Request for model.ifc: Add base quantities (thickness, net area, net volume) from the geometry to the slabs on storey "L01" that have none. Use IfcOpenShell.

First a look at what the model holds.

```python
import ifcopenshell
import ifcopenshell.util.element
import ifcopenshell.util.unit

model = ifcopenshell.open("model.ifc")
print(model.schema)
for unit_type in ("LENGTHUNIT", "AREAUNIT", "VOLUMEUNIT"):
    print(unit_type, ifcopenshell.util.unit.calculate_unit_scale(model, unit_type))
storey = next(s for s in model.by_type("IfcBuildingStorey") if s.Name == "L01")
slabs = [e for e in ifcopenshell.util.element.get_decomposition(storey) if e.is_a("IfcSlab")]
for e in sorted(slabs, key=lambda e: e.id()):
    print(e.id(), e.is_a(), e.Name, list(ifcopenshell.util.element.get_psets(e, qtos_only=True)), sep=" | ")
```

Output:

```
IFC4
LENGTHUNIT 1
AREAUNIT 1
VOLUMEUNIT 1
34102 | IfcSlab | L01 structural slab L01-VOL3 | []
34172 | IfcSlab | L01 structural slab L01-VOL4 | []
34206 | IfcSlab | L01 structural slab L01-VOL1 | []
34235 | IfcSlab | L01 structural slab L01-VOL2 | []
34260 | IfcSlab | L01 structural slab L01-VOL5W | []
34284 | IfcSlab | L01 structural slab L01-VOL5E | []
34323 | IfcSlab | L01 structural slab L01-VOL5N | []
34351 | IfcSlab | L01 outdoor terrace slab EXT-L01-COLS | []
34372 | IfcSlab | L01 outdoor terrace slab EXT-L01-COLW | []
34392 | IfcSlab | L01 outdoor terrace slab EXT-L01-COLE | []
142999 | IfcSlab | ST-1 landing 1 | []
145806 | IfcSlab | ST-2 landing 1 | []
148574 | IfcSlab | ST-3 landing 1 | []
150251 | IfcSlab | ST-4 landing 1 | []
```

```python
import ifcopenshell
import ifcopenshell.api.pset
import ifcopenshell.geom
import ifcopenshell.util.element
import ifcopenshell.util.shape
import ifcopenshell.util.unit

model = ifcopenshell.open("model.ifc")
unit_scale = ifcopenshell.util.unit.calculate_unit_scale(model)
area_scale = ifcopenshell.util.unit.calculate_unit_scale(model, "AREAUNIT")
volume_scale = ifcopenshell.util.unit.calculate_unit_scale(model, "VOLUMEUNIT")
settings = ifcopenshell.geom.settings()

storey = next(s for s in model.by_type("IfcBuildingStorey") if s.Name == "L01")
slabs = [e for e in ifcopenshell.util.element.get_decomposition(storey) if e.is_a("IfcSlab")]

for e in sorted(slabs, key=lambda e: e.id()):
    if ifcopenshell.util.element.get_psets(e, qtos_only=True, should_inherit=False):
        continue
    # Geometry comes back in metres, in the element's own axes.
    shape = ifcopenshell.geom.create_shape(settings, e)
    values = {
        "Width": ifcopenshell.util.shape.get_z(shape.geometry) / unit_scale,
        "NetArea": ifcopenshell.util.shape.get_footprint_area(shape.geometry) / area_scale,
        "NetVolume": ifcopenshell.util.shape.get_volume(shape.geometry) / volume_scale,
    }
    qto = ifcopenshell.api.pset.add_qto(model, product=e, name="Qto_SlabBaseQuantities")
    ifcopenshell.api.pset.edit_qto(model, qto=qto, properties=values)
    print(e.id(), {k: round(v, 3) for k, v in values.items()})

model.write("model_v2.ifc")
```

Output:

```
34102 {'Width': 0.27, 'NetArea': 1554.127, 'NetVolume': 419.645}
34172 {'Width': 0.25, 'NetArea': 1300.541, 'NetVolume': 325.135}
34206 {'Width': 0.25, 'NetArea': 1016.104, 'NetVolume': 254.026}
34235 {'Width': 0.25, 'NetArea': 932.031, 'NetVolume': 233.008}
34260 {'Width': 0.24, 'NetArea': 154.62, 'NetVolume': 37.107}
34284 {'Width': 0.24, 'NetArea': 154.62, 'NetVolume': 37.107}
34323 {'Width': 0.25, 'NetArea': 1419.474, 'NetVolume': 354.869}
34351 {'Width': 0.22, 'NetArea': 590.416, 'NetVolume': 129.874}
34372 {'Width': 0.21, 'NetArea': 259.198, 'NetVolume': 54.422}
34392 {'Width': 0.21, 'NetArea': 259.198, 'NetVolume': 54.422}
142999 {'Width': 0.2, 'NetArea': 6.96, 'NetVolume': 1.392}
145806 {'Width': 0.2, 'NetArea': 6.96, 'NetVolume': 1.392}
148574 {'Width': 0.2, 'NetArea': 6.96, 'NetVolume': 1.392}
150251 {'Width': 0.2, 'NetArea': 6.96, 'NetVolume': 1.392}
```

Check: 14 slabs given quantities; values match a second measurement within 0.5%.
